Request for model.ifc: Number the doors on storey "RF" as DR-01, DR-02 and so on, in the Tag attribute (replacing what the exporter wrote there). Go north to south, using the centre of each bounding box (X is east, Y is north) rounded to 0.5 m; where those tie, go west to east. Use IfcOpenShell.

First a look at what the model holds.

```python
import ifcopenshell
import ifcopenshell.util.element
import ifcopenshell.util.placement

model = ifcopenshell.open("model.ifc")
print(model.schema)
storey = next(s for s in model.by_type("IfcBuildingStorey") if s.Name == "RF")
doors = [e for e in ifcopenshell.util.element.get_decomposition(storey) if e.is_a("IfcDoor")]
for e in sorted(doors, key=lambda e: e.id()):
    origin = ifcopenshell.util.placement.get_local_placement(e.ObjectPlacement)[:3, 3]
    print(e.id(), e.Tag, e.Name, origin.round(2) + 0.0, sep=" | ")
```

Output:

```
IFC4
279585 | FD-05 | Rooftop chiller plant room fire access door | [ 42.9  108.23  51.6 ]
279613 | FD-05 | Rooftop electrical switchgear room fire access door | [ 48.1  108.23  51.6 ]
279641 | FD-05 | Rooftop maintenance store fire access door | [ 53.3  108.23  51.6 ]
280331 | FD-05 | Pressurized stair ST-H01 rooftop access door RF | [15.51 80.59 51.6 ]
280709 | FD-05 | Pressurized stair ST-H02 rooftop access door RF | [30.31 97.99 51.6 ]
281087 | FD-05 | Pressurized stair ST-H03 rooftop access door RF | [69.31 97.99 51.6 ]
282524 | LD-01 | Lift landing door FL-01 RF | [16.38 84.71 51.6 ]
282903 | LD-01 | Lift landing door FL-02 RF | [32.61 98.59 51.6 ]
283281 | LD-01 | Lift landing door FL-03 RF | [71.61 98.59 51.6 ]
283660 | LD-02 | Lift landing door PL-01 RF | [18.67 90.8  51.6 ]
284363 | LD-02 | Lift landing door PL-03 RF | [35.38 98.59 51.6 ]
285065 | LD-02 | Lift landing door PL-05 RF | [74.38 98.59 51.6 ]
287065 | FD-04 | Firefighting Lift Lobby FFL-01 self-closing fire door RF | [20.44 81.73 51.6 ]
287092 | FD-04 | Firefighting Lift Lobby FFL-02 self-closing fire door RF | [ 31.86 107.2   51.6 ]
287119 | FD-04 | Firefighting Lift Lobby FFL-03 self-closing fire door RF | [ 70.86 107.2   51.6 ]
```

```python
import ifcopenshell
import ifcopenshell.geom
import ifcopenshell.util.element
import ifcopenshell.util.shape

model = ifcopenshell.open("model.ifc")
settings = ifcopenshell.geom.settings()
settings.set("use-world-coords", True)


def centre(element):
    shape = ifcopenshell.geom.create_shape(settings, element)
    return ifcopenshell.util.shape.get_bbox_centroid(shape.geometry)


storey = next(s for s in model.by_type("IfcBuildingStorey") if s.Name == "RF")
doors = [e for e in ifcopenshell.util.element.get_decomposition(storey) if e.is_a("IfcDoor")]

# Insertion points can sit at a corner or the storey origin, so sort by the geometry (in metres).
centres = {e: centre(e) for e in doors}
doors.sort(key=lambda e: (-round(centres[e][1] / 0.5), centres[e][0]))

for i, e in enumerate(doors, start=1):
    number = f"DR-{i:02d}"
    e.Tag = number
    print(e.id(), number)

model.write("model_edited.ifc")
```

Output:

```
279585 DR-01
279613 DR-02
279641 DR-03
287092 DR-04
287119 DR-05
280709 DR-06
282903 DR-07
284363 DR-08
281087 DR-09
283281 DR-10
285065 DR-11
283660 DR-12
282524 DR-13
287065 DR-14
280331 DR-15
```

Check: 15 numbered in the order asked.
